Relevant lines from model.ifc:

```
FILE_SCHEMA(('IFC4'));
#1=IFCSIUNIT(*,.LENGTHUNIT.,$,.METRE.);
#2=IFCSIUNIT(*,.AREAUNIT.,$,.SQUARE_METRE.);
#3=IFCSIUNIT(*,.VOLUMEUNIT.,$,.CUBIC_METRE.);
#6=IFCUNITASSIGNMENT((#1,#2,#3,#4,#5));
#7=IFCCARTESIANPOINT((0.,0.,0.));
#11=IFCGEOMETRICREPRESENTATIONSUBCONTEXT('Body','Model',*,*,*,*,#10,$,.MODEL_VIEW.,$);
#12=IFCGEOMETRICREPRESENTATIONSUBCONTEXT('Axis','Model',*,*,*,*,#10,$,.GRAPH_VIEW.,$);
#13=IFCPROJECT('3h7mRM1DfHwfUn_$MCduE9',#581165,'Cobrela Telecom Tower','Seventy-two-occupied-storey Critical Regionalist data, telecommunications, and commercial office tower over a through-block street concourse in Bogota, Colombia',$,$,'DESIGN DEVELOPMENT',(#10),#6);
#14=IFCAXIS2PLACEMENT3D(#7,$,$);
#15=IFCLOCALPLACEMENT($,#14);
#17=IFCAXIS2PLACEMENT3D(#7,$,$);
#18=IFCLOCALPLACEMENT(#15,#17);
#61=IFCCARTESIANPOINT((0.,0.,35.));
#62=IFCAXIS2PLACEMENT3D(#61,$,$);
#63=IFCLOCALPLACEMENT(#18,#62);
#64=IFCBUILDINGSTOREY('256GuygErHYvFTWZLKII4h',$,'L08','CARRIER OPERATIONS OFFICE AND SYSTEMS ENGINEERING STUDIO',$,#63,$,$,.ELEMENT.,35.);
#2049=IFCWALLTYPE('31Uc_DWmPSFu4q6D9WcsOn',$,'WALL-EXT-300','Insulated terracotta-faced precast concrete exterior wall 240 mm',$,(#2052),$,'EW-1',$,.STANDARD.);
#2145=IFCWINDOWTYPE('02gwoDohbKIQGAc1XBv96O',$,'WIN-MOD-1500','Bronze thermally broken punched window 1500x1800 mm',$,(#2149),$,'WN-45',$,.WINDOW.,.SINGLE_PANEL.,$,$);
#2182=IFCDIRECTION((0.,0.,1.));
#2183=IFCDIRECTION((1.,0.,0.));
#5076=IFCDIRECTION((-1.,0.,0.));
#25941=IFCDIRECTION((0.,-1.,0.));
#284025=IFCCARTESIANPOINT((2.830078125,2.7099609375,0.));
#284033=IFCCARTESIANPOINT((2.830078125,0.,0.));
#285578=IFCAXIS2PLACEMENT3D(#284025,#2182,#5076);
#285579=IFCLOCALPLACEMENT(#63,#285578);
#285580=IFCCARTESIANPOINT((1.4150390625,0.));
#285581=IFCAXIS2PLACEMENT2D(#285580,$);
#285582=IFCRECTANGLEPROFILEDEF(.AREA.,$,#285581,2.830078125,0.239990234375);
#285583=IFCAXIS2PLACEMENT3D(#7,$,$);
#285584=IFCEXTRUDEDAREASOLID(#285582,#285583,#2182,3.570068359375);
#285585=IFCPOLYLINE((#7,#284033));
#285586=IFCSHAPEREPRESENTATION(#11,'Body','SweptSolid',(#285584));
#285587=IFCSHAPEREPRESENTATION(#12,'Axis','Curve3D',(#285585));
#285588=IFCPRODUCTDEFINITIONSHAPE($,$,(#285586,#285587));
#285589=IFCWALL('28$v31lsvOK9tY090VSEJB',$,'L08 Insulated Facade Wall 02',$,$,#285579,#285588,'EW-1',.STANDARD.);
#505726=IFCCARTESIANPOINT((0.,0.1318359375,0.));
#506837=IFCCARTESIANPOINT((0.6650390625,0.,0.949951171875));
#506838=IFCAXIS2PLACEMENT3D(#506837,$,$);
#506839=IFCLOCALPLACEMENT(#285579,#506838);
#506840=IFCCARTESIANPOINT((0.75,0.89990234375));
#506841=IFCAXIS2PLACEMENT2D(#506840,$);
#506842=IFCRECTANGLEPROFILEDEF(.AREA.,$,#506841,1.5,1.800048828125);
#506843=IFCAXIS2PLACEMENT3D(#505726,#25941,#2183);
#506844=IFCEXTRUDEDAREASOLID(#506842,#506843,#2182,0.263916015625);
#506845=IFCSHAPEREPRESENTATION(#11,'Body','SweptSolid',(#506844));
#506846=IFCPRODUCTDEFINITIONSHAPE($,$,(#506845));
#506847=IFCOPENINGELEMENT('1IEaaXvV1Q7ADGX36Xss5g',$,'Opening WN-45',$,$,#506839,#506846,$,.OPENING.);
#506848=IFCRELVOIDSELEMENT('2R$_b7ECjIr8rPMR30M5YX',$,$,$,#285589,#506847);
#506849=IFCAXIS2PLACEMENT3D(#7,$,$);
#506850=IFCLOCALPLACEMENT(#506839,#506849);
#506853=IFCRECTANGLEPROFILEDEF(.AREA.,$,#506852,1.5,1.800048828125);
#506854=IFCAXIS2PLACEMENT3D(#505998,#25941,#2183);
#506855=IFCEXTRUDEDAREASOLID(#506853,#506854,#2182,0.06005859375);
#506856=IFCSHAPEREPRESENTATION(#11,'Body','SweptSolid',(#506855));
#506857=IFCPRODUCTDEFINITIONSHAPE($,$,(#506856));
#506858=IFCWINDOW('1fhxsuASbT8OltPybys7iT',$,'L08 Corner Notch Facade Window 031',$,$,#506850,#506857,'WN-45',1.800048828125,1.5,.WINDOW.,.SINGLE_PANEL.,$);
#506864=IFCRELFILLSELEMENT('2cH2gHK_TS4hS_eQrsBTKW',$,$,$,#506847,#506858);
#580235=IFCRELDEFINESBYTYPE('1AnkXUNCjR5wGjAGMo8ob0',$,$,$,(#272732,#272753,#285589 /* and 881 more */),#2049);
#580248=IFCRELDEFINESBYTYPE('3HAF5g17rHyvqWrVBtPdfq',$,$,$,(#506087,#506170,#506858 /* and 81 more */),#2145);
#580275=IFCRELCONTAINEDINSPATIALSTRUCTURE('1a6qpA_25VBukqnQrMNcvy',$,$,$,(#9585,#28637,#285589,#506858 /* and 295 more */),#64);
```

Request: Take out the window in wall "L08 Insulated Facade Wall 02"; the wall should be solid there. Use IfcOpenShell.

```python
import ifcopenshell
import ifcopenshell.api.feature
import ifcopenshell.api.root
import ifcopenshell.geom
import ifcopenshell.util.shape

model = ifcopenshell.open("model.ifc")
settings = ifcopenshell.geom.settings()


def volume(element):
    """Net volume in cubic metres, openings subtracted."""
    shape = ifcopenshell.geom.create_shape(settings, element)
    return ifcopenshell.util.shape.get_volume(shape.geometry)


window = model.by_guid("1fhxsuASbT8OltPybys7iT")
opening = window.FillsVoids[0].RelatingOpeningElement
wall = opening.VoidsElements[0].RelatingBuildingElement
before = volume(wall)

ifcopenshell.api.root.remove_product(model, product=window)
ifcopenshell.api.feature.remove_feature(model, feature=opening)

after = volume(wall)

print(f"wall volume {before:.3f} -> {after:.3f} m3")

model.write("model_edited.ifc")
```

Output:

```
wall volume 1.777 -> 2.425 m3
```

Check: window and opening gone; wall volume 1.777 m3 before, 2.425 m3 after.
